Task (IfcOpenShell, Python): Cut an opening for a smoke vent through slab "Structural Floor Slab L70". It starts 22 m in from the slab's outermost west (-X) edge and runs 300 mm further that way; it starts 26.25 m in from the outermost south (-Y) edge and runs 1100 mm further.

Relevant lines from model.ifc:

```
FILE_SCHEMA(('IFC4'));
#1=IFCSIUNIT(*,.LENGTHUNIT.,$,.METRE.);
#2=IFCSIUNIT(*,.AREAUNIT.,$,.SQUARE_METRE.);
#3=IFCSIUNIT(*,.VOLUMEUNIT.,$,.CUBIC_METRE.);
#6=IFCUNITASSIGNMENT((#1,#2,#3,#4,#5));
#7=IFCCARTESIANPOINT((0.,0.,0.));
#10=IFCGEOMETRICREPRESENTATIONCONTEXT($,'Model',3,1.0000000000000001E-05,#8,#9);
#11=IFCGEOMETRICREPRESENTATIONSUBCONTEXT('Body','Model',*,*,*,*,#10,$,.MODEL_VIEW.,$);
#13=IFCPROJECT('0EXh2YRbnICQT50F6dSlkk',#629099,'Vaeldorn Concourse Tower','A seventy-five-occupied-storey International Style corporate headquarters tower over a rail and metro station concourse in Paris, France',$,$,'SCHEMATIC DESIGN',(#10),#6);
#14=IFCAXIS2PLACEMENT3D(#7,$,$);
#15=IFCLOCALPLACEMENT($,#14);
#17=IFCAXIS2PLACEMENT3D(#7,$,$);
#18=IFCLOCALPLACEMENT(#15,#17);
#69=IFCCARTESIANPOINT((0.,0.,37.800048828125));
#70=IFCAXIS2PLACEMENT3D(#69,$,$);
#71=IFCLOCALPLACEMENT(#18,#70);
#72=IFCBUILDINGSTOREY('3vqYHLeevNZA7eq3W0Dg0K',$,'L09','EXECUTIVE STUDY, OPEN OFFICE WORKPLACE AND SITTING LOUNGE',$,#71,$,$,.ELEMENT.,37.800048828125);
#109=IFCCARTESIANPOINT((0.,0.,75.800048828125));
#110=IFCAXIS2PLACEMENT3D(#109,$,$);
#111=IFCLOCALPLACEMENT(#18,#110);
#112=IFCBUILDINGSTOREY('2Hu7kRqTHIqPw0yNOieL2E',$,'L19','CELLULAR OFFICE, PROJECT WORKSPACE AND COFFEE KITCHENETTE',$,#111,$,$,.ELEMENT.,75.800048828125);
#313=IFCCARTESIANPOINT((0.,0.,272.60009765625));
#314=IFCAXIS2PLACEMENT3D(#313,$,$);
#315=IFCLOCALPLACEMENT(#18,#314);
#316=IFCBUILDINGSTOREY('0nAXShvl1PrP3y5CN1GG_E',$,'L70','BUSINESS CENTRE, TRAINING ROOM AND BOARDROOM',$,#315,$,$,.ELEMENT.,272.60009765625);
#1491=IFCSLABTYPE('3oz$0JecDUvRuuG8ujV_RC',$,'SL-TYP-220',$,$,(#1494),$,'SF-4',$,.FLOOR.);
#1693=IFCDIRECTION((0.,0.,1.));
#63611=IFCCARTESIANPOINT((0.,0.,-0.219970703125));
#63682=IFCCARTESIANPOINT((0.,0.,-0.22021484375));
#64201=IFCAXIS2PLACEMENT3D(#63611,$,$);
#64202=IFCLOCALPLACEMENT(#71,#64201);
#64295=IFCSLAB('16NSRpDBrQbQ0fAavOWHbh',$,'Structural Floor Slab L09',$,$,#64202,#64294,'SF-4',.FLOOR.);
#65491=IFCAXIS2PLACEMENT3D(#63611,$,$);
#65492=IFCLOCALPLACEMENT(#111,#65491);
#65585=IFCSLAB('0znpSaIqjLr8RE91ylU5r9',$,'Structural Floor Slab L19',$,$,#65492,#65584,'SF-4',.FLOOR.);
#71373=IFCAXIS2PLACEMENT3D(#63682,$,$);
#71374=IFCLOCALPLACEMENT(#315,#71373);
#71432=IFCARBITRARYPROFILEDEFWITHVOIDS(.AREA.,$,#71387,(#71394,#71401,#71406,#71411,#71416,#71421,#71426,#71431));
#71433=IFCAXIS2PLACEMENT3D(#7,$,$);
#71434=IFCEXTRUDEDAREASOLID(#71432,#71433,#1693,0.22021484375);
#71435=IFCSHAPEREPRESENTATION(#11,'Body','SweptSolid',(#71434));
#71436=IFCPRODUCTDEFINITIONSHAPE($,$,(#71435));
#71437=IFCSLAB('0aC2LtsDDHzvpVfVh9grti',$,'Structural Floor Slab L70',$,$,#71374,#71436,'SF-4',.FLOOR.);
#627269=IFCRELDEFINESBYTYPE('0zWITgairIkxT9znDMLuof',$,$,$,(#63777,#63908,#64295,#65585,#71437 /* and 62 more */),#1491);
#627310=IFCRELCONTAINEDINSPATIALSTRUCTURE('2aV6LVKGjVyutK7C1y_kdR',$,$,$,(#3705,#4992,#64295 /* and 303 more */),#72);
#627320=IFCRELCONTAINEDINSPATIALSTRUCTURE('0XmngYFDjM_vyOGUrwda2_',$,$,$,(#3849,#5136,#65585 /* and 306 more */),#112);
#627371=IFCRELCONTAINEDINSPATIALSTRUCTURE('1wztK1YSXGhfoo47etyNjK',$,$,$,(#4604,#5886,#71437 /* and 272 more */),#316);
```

```python
import numpy as np
import ifcopenshell
import ifcopenshell.api.feature
import ifcopenshell.api.geometry
import ifcopenshell.api.root
import ifcopenshell.geom
import ifcopenshell.util.placement
import ifcopenshell.util.representation
import ifcopenshell.util.shape
import ifcopenshell.util.unit

model = ifcopenshell.open("model.ifc")
unit_scale = ifcopenshell.util.unit.calculate_unit_scale(model)
settings = ifcopenshell.geom.settings()


def volume(element):
    """Net volume in cubic metres, openings subtracted."""
    shape = ifcopenshell.geom.create_shape(settings, element)
    return ifcopenshell.util.shape.get_volume(shape.geometry)


slab = model.by_guid("0aC2LtsDDHzvpVfVh9grti")
before = volume(slab)

# Extent in the slab's own axes, in metres. The edges named are its -X and -Y sides.
slab_shape = ifcopenshell.geom.create_shape(settings, slab)
vertices = ifcopenshell.util.shape.get_vertices(slab_shape.geometry)
x_min, y_min, bottom = vertices.min(axis=0)
top = vertices[:, 2].max()

opening = ifcopenshell.api.root.create_entity(model, ifc_class="IfcOpeningElement", name="Smoke vent opening", predefined_type="OPENING")
context = ifcopenshell.util.representation.get_context(model, "Model", "Body", "MODEL_VIEW")
width, depth = 0.3, 1.1
outline = [(0.0, 0.0), (width, 0.0), (width, depth), (0.0, depth), (0.0, 0.0)]
# Overshoot both faces by 50 mm so the cut is clean.
shape = ifcopenshell.api.geometry.add_slab_representation(
    model, context=context, depth=top - bottom + 0.1, polyline=outline
)
ifcopenshell.api.geometry.assign_representation(model, product=opening, representation=shape)

matrix = ifcopenshell.util.placement.get_local_placement(slab.ObjectPlacement)
matrix[:, 3] = matrix @ np.append(np.array([x_min + 22, y_min + 26.25, bottom - 0.05]) / unit_scale, 1.0)
ifcopenshell.api.geometry.edit_object_placement(model, product=opening, matrix=matrix, is_si=False)
ifcopenshell.api.feature.add_feature(model, feature=opening, element=slab)

after = volume(slab)

print(f"slab volume {before:.3f} -> {after:.3f} m3")

model.write("model_rev.ifc")
```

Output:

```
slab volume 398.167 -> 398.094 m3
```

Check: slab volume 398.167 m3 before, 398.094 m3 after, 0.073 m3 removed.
